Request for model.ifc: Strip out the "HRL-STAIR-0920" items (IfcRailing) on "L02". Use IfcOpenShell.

First a look at what the model holds.

```python
import ifcopenshell
import ifcopenshell.util.element

model = ifcopenshell.open("model.ifc")
print(model.schema)
storey = next(s for s in model.by_type("IfcBuildingStorey") if s.Name == "L02")
railings = [e for e in ifcopenshell.util.element.get_decomposition(storey) if e.is_a("IfcRailing")]
seen = {}
for e in railings:
    element_type = ifcopenshell.util.element.get_type(e)
    name = element_type.Name if element_type not in (None, e) else None
    seen[name] = seen.get(name, 0) + 1
for name, count in sorted(seen.items(), key=str):
    print(count, "x", name)
```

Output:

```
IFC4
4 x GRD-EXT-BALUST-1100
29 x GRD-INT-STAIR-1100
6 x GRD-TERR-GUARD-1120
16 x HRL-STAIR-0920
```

```python
import ifcopenshell
import ifcopenshell.api.root
import ifcopenshell.util.element

model = ifcopenshell.open("model.ifc")

storey = next(s for s in model.by_type("IfcBuildingStorey") if s.Name == "L02")
railings = [e for e in ifcopenshell.util.element.get_decomposition(storey) if e.is_a("IfcRailing")]
targets = [e for e in railings if (t := ifcopenshell.util.element.get_type(e)) not in (None, e) and t.Name == "HRL-STAIR-0920"]

for e in targets:
    ifcopenshell.api.root.remove_product(model, product=e)
print(len(targets), "removed")

model.write("model-out.ifc")
```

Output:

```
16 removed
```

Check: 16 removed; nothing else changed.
